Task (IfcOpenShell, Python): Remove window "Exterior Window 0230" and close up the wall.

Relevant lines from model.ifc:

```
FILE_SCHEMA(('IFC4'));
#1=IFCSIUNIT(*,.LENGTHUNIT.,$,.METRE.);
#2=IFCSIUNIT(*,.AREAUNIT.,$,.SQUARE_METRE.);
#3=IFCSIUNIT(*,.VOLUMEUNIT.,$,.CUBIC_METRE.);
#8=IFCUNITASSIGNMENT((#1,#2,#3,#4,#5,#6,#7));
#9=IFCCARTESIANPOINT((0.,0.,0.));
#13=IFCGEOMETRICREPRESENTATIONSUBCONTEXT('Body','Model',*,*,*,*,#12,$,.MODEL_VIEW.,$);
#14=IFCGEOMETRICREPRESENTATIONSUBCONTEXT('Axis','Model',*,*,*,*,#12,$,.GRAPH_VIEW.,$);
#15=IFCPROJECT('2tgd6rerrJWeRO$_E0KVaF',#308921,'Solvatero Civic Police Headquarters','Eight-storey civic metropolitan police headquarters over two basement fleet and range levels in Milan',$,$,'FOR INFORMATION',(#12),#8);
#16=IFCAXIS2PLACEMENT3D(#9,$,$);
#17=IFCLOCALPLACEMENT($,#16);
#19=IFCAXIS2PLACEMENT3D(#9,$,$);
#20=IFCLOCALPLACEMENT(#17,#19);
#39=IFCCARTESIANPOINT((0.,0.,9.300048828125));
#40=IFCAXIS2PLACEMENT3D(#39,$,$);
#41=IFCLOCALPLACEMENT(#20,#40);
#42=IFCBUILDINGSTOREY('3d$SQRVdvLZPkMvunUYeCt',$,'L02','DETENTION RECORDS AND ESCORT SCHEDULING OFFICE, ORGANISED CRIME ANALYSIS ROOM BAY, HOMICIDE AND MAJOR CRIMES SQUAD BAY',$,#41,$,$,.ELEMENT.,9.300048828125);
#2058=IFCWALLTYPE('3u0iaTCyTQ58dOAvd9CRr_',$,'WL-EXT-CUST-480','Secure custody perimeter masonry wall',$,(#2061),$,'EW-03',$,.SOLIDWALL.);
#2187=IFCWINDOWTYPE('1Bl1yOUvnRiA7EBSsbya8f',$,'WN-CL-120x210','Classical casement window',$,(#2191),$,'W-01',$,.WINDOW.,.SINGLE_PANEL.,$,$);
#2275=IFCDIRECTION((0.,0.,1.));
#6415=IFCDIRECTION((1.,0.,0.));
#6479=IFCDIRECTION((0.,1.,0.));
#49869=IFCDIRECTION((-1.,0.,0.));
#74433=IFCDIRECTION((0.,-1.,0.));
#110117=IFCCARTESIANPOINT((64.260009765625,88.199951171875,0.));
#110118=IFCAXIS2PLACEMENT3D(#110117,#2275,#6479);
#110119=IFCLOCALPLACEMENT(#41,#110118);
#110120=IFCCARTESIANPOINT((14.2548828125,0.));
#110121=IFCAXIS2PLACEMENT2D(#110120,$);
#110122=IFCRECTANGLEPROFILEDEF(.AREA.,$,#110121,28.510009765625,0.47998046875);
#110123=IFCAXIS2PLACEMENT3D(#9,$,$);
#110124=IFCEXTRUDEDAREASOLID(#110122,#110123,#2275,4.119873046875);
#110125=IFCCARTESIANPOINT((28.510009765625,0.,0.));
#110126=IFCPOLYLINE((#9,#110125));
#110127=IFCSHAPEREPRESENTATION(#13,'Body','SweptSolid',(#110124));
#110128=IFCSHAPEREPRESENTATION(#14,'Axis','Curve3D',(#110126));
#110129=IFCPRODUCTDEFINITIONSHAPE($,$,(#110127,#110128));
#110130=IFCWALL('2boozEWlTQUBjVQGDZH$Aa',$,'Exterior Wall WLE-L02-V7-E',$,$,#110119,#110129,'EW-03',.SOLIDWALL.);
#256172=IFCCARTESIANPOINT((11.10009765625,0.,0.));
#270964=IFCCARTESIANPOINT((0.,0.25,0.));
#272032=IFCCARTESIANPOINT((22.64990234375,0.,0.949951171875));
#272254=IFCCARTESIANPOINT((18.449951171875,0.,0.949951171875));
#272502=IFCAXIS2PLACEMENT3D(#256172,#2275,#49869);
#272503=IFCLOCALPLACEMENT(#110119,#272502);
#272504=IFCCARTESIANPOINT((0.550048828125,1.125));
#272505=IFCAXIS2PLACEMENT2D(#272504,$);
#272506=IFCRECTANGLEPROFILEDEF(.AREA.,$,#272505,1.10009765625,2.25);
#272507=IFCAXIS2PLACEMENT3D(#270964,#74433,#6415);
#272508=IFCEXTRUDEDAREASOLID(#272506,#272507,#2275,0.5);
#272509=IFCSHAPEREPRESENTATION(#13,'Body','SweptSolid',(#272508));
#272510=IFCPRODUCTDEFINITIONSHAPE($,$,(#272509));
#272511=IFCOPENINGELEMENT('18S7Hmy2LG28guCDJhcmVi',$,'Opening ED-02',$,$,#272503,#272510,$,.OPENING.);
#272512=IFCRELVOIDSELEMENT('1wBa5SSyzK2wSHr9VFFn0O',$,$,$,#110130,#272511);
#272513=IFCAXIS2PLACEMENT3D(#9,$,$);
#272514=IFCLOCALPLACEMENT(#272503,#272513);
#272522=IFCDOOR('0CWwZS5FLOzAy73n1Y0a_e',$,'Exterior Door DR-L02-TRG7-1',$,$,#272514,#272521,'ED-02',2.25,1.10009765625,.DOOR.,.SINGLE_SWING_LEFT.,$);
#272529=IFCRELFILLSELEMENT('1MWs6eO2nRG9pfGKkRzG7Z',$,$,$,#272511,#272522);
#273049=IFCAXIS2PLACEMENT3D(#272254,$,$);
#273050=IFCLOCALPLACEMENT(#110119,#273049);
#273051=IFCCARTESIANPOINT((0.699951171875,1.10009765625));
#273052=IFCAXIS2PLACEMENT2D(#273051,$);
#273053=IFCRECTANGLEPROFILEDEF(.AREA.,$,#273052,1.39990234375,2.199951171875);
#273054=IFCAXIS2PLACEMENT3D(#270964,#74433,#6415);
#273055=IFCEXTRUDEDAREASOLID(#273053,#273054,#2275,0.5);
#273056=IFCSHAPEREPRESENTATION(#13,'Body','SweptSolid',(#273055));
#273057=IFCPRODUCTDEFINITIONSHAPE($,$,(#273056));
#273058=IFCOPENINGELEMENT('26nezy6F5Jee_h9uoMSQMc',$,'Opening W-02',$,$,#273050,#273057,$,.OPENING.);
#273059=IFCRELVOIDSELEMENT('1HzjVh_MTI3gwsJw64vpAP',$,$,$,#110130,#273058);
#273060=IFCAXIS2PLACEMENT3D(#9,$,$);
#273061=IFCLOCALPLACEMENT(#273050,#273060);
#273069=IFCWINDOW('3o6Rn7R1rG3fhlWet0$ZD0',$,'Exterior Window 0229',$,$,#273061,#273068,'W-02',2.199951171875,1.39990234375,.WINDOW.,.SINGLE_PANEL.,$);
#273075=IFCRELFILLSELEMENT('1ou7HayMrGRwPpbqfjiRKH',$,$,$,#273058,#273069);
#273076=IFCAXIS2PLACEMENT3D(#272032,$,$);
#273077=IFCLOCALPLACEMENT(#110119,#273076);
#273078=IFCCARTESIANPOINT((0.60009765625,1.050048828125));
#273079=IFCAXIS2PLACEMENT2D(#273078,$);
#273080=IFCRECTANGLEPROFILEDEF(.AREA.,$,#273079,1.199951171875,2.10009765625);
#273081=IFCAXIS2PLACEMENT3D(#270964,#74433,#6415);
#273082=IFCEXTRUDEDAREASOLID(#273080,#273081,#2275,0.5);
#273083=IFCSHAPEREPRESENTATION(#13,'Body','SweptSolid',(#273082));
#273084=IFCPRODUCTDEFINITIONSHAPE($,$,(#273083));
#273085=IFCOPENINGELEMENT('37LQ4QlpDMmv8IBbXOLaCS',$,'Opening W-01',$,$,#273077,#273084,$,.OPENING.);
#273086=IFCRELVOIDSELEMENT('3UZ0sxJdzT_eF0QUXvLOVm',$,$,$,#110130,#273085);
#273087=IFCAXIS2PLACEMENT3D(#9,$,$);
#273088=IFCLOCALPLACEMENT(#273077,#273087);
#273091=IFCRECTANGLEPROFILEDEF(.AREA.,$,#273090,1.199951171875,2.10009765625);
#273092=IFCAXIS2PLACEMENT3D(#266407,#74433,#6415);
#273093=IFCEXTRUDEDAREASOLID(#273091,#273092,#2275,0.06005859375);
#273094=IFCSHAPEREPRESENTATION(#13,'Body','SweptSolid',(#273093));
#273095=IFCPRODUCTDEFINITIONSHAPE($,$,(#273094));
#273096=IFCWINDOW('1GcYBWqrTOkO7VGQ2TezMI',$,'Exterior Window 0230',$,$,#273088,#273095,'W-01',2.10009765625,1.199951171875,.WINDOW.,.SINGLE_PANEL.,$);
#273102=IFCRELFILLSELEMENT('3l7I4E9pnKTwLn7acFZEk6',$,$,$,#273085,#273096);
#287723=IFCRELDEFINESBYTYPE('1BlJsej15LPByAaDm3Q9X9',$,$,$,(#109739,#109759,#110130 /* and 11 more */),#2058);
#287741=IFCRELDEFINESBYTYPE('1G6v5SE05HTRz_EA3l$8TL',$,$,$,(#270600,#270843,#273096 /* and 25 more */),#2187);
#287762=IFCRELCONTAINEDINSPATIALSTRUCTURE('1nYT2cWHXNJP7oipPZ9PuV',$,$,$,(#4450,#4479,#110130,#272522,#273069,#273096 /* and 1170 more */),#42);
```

```python
import ifcopenshell
import ifcopenshell.api.feature
import ifcopenshell.api.root
import ifcopenshell.geom
import ifcopenshell.util.shape

model = ifcopenshell.open("model.ifc")
settings = ifcopenshell.geom.settings()


def volume(element):
    """Net volume in cubic metres, openings subtracted."""
    shape = ifcopenshell.geom.create_shape(settings, element)
    return ifcopenshell.util.shape.get_volume(shape.geometry)


window = model.by_id(273096)
opening = window.FillsVoids[0].RelatingOpeningElement
wall = opening.VoidsElements[0].RelatingBuildingElement
before = volume(wall)

ifcopenshell.api.root.remove_product(model, product=window)
ifcopenshell.api.feature.remove_feature(model, feature=opening)

after = volume(wall)

print(f"wall volume {before:.3f} -> {after:.3f} m3")

model.write("model_rev.ifc")
```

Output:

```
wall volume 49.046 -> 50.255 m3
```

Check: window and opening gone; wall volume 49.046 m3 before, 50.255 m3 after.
